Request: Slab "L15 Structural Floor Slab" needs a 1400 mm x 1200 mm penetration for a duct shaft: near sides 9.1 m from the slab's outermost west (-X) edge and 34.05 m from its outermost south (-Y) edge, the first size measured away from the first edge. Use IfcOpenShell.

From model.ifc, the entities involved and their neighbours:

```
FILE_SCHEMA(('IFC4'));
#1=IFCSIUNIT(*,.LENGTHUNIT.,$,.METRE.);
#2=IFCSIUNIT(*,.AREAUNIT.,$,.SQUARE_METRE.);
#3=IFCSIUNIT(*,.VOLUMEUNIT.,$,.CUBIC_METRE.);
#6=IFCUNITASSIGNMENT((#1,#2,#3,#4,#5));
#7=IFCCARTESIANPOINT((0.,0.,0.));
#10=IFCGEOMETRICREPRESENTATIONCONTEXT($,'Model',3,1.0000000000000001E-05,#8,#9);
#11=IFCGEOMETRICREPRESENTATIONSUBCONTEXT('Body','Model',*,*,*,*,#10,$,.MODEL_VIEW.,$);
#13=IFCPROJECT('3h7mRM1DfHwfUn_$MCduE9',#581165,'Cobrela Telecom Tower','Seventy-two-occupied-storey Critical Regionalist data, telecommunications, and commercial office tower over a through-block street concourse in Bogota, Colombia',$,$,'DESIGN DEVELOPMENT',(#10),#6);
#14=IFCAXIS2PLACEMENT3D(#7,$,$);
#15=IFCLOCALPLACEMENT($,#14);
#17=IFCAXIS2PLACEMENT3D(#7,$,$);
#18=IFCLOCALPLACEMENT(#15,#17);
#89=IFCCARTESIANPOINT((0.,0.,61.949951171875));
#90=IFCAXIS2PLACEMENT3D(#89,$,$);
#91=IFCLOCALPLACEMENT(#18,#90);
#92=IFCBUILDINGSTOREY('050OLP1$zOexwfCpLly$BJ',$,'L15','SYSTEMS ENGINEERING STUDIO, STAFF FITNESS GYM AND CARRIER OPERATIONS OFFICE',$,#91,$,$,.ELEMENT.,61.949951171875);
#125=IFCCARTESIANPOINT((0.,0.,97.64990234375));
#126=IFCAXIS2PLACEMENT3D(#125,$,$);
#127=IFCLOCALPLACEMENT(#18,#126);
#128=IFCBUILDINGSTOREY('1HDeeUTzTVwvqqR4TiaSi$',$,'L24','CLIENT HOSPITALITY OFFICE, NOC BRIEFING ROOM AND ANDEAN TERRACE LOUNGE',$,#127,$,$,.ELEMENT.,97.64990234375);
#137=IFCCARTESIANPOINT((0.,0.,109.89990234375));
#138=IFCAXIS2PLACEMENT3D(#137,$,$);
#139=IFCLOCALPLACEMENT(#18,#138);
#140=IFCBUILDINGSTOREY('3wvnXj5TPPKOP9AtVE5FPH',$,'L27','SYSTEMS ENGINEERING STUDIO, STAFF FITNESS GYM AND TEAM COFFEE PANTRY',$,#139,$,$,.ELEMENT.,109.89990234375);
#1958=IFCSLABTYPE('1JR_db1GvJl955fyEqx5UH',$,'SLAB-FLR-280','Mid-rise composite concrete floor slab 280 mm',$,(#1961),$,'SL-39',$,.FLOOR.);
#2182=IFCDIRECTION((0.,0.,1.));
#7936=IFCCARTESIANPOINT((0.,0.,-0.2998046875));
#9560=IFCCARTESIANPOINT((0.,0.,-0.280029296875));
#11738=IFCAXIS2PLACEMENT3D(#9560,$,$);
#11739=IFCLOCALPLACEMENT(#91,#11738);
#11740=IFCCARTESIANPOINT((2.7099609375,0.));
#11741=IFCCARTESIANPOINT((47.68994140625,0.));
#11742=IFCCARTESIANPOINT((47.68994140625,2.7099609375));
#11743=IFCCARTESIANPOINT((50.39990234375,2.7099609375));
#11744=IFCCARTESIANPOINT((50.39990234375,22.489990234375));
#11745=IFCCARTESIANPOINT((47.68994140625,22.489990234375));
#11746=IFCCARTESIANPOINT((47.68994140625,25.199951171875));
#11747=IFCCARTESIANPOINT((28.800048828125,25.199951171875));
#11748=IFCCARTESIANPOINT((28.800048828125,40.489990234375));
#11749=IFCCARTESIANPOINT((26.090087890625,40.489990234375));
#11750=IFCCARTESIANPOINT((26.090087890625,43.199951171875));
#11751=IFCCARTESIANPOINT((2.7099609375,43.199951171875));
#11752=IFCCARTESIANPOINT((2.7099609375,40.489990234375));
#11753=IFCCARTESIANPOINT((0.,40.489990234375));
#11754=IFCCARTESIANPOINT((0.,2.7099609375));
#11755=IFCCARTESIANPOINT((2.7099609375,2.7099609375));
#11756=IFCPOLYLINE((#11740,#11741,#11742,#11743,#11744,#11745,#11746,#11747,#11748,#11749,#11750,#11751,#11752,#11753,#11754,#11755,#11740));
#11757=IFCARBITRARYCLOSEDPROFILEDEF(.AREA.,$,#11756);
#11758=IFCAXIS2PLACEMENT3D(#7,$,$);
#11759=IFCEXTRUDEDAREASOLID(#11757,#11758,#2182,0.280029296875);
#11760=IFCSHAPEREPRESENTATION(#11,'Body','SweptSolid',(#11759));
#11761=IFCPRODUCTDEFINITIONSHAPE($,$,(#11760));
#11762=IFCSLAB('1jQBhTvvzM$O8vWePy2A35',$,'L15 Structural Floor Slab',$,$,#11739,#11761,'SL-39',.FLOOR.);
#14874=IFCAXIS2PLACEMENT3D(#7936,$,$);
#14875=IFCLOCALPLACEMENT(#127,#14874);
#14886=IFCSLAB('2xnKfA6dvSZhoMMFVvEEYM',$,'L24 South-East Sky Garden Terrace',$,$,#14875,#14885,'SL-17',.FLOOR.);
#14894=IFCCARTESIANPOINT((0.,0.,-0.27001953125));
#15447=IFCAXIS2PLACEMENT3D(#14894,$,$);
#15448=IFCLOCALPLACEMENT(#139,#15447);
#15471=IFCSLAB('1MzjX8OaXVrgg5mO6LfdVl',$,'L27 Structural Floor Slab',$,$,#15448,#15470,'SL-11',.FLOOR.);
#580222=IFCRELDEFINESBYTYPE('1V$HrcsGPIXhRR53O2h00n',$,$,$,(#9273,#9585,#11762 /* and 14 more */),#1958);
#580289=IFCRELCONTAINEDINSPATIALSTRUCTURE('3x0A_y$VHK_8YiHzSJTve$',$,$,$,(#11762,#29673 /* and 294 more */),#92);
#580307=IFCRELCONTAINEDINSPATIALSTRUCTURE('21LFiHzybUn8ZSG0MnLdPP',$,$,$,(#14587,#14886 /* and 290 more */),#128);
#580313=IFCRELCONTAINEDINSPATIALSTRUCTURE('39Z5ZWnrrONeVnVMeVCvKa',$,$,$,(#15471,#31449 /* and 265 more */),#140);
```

```python
import numpy as np
import ifcopenshell
import ifcopenshell.api.feature
import ifcopenshell.api.geometry
import ifcopenshell.api.root
import ifcopenshell.geom
import ifcopenshell.util.placement
import ifcopenshell.util.representation
import ifcopenshell.util.shape
import ifcopenshell.util.unit

model = ifcopenshell.open("model.ifc")
unit_scale = ifcopenshell.util.unit.calculate_unit_scale(model)
settings = ifcopenshell.geom.settings()


def volume(element):
    """Net volume in cubic metres, openings subtracted."""
    shape = ifcopenshell.geom.create_shape(settings, element)
    return ifcopenshell.util.shape.get_volume(shape.geometry)


slab = model.by_id(11762)
before = volume(slab)

# Extent in the slab's own axes, in metres. The edges named are its -X and -Y sides.
slab_shape = ifcopenshell.geom.create_shape(settings, slab)
vertices = ifcopenshell.util.shape.get_vertices(slab_shape.geometry)
x_min, y_min, bottom = vertices.min(axis=0)
top = vertices[:, 2].max()

opening = ifcopenshell.api.root.create_entity(model, ifc_class="IfcOpeningElement", name="Duct shaft opening", predefined_type="OPENING")
context = ifcopenshell.util.representation.get_context(model, "Model", "Body", "MODEL_VIEW")
width, depth = 1.4, 1.2
outline = [(0.0, 0.0), (width, 0.0), (width, depth), (0.0, depth), (0.0, 0.0)]
# Overshoot both faces by 50 mm so the cut is clean.
shape = ifcopenshell.api.geometry.add_slab_representation(
    model, context=context, depth=top - bottom + 0.1, polyline=outline
)
ifcopenshell.api.geometry.assign_representation(model, product=opening, representation=shape)

matrix = ifcopenshell.util.placement.get_local_placement(slab.ObjectPlacement)
matrix[:, 3] = matrix @ np.append(np.array([x_min + 9.1, y_min + 34.05, bottom - 0.05]) / unit_scale, 1.0)
ifcopenshell.api.geometry.edit_object_placement(model, product=opening, matrix=matrix, is_si=False)
ifcopenshell.api.feature.add_feature(model, feature=opening, element=slab)

after = volume(slab)

print(f"slab volume {before:.3f} -> {after:.3f} m3")

model.write("model_v2.ifc")
```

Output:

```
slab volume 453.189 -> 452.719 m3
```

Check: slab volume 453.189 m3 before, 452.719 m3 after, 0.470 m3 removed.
